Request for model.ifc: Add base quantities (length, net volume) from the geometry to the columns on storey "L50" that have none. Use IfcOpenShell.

First a look at what the model holds.

```python
import ifcopenshell
import ifcopenshell.util.element
import ifcopenshell.util.unit

model = ifcopenshell.open("model.ifc")
print(model.schema)
for unit_type in ("LENGTHUNIT", "AREAUNIT", "VOLUMEUNIT"):
    print(unit_type, ifcopenshell.util.unit.calculate_unit_scale(model, unit_type))
storey = next(s for s in model.by_type("IfcBuildingStorey") if s.Name == "L50")
columns = [e for e in ifcopenshell.util.element.get_decomposition(storey) if e.is_a("IfcColumn")]
for e in sorted(columns, key=lambda e: e.id()):
    print(e.id(), e.is_a(), e.Name, list(ifcopenshell.util.element.get_psets(e, qtos_only=True)), sep=" | ")
```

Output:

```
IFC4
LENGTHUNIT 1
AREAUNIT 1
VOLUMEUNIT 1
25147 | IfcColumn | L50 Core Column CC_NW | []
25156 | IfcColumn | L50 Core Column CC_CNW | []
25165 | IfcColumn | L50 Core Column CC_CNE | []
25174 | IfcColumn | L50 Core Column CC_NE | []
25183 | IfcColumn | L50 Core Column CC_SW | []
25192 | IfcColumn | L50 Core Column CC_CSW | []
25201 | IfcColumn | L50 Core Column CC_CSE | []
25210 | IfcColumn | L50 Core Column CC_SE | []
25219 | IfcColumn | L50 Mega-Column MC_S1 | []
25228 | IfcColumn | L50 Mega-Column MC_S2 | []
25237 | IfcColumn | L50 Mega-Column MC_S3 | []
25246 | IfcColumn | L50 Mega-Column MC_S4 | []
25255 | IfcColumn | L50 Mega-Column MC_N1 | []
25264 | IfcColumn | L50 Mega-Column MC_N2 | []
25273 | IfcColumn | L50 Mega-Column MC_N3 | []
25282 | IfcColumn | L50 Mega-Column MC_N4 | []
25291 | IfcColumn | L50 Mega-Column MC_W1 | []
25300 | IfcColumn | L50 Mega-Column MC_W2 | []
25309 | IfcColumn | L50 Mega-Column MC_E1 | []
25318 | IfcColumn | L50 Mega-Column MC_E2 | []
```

```python
import ifcopenshell
import ifcopenshell.api.pset
import ifcopenshell.geom
import ifcopenshell.util.element
import ifcopenshell.util.shape
import ifcopenshell.util.unit

model = ifcopenshell.open("model.ifc")
unit_scale = ifcopenshell.util.unit.calculate_unit_scale(model)
volume_scale = ifcopenshell.util.unit.calculate_unit_scale(model, "VOLUMEUNIT")
settings = ifcopenshell.geom.settings()

storey = next(s for s in model.by_type("IfcBuildingStorey") if s.Name == "L50")
columns = [e for e in ifcopenshell.util.element.get_decomposition(storey) if e.is_a("IfcColumn")]

for e in sorted(columns, key=lambda e: e.id()):
    if ifcopenshell.util.element.get_psets(e, qtos_only=True, should_inherit=False):
        continue
    # Geometry comes back in metres, in the element's own axes.
    shape = ifcopenshell.geom.create_shape(settings, e)
    values = {
        "Length": ifcopenshell.util.shape.get_z(shape.geometry) / unit_scale,
        "NetVolume": ifcopenshell.util.shape.get_volume(shape.geometry) / volume_scale,
    }
    qto = ifcopenshell.api.pset.add_qto(model, product=e, name="Qto_ColumnBaseQuantities")
    ifcopenshell.api.pset.edit_qto(model, qto=qto, properties=values)
    print(e.id(), {k: round(v, 3) for k, v in values.items()})

model.write("model_rev.ifc")
```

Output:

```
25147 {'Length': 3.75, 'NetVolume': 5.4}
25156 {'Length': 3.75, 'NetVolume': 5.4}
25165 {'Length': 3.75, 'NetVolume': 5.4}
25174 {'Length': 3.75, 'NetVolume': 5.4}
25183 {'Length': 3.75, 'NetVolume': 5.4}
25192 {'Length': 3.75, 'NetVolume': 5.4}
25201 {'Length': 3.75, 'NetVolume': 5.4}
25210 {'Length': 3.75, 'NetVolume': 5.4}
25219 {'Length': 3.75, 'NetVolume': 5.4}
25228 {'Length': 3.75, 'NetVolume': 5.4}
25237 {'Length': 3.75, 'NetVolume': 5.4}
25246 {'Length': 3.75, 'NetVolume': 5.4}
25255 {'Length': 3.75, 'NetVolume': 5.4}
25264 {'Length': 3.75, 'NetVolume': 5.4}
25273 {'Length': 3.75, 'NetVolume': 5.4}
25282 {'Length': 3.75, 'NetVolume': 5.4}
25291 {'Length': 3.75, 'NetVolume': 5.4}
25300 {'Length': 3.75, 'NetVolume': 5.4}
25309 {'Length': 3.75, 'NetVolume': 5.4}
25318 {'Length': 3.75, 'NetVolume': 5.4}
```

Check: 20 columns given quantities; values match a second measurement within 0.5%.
